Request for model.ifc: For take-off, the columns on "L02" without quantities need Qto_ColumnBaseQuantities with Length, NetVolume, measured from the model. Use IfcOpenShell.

First a look at what the model holds.

```python
import ifcopenshell
import ifcopenshell.util.element
import ifcopenshell.util.unit

model = ifcopenshell.open("model.ifc")
print(model.schema)
for unit_type in ("LENGTHUNIT", "AREAUNIT", "VOLUMEUNIT"):
    print(unit_type, ifcopenshell.util.unit.calculate_unit_scale(model, unit_type))
storey = next(s for s in model.by_type("IfcBuildingStorey") if s.Name == "L02")
columns = [e for e in ifcopenshell.util.element.get_decomposition(storey) if e.is_a("IfcColumn")]
for e in sorted(columns, key=lambda e: e.id()):
    print(e.id(), e.is_a(), e.Name, list(ifcopenshell.util.element.get_psets(e, qtos_only=True)), sep=" | ")
```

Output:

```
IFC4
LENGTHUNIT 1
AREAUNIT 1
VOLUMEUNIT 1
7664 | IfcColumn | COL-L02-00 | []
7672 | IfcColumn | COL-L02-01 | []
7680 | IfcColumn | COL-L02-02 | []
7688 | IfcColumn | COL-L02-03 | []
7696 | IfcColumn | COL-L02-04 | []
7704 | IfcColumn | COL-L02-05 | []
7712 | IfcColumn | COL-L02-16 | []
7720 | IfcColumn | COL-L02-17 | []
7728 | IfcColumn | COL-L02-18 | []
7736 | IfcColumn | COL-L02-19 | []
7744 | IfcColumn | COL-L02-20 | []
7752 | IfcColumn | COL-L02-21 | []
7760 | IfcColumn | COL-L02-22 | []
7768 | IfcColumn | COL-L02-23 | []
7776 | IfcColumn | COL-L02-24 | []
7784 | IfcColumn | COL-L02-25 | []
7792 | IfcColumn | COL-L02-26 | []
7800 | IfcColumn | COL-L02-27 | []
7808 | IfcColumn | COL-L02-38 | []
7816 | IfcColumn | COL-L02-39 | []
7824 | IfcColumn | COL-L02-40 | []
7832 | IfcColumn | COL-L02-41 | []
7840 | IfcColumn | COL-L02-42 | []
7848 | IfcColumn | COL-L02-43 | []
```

```python
import ifcopenshell
import ifcopenshell.api.pset
import ifcopenshell.geom
import ifcopenshell.util.element
import ifcopenshell.util.shape
import ifcopenshell.util.unit

model = ifcopenshell.open("model.ifc")
unit_scale = ifcopenshell.util.unit.calculate_unit_scale(model)
volume_scale = ifcopenshell.util.unit.calculate_unit_scale(model, "VOLUMEUNIT")
settings = ifcopenshell.geom.settings()

storey = next(s for s in model.by_type("IfcBuildingStorey") if s.Name == "L02")
columns = [e for e in ifcopenshell.util.element.get_decomposition(storey) if e.is_a("IfcColumn")]

for e in sorted(columns, key=lambda e: e.id()):
    if ifcopenshell.util.element.get_psets(e, qtos_only=True, should_inherit=False):
        continue
    # Geometry comes back in metres, in the element's own axes.
    shape = ifcopenshell.geom.create_shape(settings, e)
    values = {
        "Length": ifcopenshell.util.shape.get_z(shape.geometry) / unit_scale,
        "NetVolume": ifcopenshell.util.shape.get_volume(shape.geometry) / volume_scale,
    }
    qto = ifcopenshell.api.pset.add_qto(model, product=e, name="Qto_ColumnBaseQuantities")
    ifcopenshell.api.pset.edit_qto(model, qto=qto, properties=values)
    print(e.id(), {k: round(v, 3) for k, v in values.items()})

model.write("model_updated.ifc")
```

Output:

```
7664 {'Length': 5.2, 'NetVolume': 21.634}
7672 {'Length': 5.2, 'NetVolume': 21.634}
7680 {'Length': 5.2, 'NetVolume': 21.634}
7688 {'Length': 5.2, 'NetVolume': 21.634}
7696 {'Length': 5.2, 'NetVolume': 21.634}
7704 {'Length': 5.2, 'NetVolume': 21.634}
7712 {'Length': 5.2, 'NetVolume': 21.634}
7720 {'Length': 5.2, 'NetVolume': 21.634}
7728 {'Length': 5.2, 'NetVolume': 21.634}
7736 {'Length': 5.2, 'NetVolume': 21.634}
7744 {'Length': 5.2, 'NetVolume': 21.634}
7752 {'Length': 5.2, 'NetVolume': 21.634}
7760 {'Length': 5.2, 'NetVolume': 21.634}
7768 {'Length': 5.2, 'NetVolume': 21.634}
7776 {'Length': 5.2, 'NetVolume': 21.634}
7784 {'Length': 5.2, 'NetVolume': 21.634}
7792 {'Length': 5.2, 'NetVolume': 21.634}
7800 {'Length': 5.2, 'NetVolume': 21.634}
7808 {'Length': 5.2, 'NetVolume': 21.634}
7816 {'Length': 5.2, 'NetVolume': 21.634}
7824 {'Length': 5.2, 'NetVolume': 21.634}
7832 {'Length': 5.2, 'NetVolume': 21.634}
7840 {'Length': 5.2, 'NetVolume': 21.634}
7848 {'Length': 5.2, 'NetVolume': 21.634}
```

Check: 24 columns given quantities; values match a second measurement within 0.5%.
